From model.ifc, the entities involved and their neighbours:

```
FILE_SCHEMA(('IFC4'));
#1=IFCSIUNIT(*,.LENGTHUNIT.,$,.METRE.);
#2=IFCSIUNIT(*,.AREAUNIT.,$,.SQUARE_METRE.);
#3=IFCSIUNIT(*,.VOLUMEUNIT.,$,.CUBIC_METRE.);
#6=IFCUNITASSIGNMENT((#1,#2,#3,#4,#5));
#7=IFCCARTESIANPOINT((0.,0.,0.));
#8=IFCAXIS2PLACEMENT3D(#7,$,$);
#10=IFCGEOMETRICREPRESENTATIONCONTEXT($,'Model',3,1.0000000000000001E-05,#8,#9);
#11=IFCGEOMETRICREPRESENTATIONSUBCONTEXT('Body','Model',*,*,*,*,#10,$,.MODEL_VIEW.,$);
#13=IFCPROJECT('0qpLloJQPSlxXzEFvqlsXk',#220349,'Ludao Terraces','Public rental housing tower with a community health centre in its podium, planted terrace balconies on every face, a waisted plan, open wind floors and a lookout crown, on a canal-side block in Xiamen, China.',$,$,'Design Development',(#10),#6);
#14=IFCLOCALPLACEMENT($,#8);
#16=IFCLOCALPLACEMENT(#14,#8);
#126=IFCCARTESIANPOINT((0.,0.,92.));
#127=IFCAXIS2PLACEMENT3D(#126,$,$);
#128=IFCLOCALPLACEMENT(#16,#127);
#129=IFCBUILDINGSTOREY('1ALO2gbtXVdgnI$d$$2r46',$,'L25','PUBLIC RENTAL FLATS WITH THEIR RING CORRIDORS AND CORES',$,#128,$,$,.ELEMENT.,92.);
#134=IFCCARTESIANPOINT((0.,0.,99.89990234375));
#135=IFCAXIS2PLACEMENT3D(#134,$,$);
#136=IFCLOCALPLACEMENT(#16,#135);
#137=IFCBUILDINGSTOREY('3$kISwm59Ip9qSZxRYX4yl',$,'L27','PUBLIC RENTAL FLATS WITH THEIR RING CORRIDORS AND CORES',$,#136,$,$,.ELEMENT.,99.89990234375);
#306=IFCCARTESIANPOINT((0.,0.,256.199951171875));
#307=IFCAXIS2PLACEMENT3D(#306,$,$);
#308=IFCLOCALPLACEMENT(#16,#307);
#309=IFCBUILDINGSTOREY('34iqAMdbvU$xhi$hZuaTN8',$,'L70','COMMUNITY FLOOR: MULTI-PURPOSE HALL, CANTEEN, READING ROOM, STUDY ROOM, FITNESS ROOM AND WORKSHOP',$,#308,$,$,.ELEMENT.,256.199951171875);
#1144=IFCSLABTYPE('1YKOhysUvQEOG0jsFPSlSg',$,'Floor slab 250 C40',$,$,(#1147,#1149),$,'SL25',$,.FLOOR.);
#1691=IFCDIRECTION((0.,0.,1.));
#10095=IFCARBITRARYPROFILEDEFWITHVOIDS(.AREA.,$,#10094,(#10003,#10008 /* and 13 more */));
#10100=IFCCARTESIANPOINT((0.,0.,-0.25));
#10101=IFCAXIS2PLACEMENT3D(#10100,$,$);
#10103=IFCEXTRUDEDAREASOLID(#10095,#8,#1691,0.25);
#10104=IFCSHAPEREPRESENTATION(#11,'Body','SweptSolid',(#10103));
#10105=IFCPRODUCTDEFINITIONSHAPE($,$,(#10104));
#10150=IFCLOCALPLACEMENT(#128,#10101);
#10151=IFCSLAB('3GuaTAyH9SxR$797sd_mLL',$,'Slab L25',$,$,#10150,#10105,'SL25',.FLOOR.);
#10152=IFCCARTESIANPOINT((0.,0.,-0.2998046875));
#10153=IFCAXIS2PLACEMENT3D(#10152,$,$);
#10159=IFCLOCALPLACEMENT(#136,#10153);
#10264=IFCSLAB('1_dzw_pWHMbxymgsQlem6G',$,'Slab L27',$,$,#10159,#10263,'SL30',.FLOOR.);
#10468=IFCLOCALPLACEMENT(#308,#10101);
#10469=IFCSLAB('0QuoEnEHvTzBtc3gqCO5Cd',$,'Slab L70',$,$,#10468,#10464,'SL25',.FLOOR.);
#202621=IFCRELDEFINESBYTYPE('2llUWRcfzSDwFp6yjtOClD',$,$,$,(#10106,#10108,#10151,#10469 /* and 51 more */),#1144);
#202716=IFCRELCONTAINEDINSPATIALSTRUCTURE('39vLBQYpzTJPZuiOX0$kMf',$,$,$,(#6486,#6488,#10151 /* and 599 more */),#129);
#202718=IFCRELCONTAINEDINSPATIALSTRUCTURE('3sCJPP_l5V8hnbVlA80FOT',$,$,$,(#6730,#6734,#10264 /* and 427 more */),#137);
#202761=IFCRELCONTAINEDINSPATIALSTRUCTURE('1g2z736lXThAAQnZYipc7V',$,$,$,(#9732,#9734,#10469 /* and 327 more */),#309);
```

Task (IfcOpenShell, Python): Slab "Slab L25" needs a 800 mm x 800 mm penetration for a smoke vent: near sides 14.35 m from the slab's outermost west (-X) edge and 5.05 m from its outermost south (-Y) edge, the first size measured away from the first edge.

```python
import numpy as np
import ifcopenshell
import ifcopenshell.api.feature
import ifcopenshell.api.geometry
import ifcopenshell.api.root
import ifcopenshell.geom
import ifcopenshell.util.placement
import ifcopenshell.util.representation
import ifcopenshell.util.shape
import ifcopenshell.util.unit

model = ifcopenshell.open("model.ifc")
unit_scale = ifcopenshell.util.unit.calculate_unit_scale(model)
settings = ifcopenshell.geom.settings()


def volume(element):
    """Net volume in cubic metres, openings subtracted."""
    shape = ifcopenshell.geom.create_shape(settings, element)
    return ifcopenshell.util.shape.get_volume(shape.geometry)


slab = model.by_guid("3GuaTAyH9SxR$797sd_mLL")
before = volume(slab)

# Extent in the slab's own axes, in metres. The edges named are its -X and -Y sides.
slab_shape = ifcopenshell.geom.create_shape(settings, slab)
vertices = ifcopenshell.util.shape.get_vertices(slab_shape.geometry)
x_min, y_min, bottom = vertices.min(axis=0)
top = vertices[:, 2].max()

opening = ifcopenshell.api.root.create_entity(model, ifc_class="IfcOpeningElement", name="Smoke vent opening", predefined_type="OPENING")
context = ifcopenshell.util.representation.get_context(model, "Model", "Body", "MODEL_VIEW")
width, depth = 0.8, 0.8
outline = [(0.0, 0.0), (width, 0.0), (width, depth), (0.0, depth), (0.0, 0.0)]
# Overshoot both faces by 50 mm so the cut is clean.
shape = ifcopenshell.api.geometry.add_slab_representation(
    model, context=context, depth=top - bottom + 0.1, polyline=outline
)
ifcopenshell.api.geometry.assign_representation(model, product=opening, representation=shape)

matrix = ifcopenshell.util.placement.get_local_placement(slab.ObjectPlacement)
matrix[:, 3] = matrix @ np.append(np.array([x_min + 14.35, y_min + 5.05, bottom - 0.05]) / unit_scale, 1.0)
ifcopenshell.api.geometry.edit_object_placement(model, product=opening, matrix=matrix, is_si=False)
ifcopenshell.api.feature.add_feature(model, feature=opening, element=slab)

after = volume(slab)

print(f"slab volume {before:.3f} -> {after:.3f} m3")

model.write("model-out.ifc")
```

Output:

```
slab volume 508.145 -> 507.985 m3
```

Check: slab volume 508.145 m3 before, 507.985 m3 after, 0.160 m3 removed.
